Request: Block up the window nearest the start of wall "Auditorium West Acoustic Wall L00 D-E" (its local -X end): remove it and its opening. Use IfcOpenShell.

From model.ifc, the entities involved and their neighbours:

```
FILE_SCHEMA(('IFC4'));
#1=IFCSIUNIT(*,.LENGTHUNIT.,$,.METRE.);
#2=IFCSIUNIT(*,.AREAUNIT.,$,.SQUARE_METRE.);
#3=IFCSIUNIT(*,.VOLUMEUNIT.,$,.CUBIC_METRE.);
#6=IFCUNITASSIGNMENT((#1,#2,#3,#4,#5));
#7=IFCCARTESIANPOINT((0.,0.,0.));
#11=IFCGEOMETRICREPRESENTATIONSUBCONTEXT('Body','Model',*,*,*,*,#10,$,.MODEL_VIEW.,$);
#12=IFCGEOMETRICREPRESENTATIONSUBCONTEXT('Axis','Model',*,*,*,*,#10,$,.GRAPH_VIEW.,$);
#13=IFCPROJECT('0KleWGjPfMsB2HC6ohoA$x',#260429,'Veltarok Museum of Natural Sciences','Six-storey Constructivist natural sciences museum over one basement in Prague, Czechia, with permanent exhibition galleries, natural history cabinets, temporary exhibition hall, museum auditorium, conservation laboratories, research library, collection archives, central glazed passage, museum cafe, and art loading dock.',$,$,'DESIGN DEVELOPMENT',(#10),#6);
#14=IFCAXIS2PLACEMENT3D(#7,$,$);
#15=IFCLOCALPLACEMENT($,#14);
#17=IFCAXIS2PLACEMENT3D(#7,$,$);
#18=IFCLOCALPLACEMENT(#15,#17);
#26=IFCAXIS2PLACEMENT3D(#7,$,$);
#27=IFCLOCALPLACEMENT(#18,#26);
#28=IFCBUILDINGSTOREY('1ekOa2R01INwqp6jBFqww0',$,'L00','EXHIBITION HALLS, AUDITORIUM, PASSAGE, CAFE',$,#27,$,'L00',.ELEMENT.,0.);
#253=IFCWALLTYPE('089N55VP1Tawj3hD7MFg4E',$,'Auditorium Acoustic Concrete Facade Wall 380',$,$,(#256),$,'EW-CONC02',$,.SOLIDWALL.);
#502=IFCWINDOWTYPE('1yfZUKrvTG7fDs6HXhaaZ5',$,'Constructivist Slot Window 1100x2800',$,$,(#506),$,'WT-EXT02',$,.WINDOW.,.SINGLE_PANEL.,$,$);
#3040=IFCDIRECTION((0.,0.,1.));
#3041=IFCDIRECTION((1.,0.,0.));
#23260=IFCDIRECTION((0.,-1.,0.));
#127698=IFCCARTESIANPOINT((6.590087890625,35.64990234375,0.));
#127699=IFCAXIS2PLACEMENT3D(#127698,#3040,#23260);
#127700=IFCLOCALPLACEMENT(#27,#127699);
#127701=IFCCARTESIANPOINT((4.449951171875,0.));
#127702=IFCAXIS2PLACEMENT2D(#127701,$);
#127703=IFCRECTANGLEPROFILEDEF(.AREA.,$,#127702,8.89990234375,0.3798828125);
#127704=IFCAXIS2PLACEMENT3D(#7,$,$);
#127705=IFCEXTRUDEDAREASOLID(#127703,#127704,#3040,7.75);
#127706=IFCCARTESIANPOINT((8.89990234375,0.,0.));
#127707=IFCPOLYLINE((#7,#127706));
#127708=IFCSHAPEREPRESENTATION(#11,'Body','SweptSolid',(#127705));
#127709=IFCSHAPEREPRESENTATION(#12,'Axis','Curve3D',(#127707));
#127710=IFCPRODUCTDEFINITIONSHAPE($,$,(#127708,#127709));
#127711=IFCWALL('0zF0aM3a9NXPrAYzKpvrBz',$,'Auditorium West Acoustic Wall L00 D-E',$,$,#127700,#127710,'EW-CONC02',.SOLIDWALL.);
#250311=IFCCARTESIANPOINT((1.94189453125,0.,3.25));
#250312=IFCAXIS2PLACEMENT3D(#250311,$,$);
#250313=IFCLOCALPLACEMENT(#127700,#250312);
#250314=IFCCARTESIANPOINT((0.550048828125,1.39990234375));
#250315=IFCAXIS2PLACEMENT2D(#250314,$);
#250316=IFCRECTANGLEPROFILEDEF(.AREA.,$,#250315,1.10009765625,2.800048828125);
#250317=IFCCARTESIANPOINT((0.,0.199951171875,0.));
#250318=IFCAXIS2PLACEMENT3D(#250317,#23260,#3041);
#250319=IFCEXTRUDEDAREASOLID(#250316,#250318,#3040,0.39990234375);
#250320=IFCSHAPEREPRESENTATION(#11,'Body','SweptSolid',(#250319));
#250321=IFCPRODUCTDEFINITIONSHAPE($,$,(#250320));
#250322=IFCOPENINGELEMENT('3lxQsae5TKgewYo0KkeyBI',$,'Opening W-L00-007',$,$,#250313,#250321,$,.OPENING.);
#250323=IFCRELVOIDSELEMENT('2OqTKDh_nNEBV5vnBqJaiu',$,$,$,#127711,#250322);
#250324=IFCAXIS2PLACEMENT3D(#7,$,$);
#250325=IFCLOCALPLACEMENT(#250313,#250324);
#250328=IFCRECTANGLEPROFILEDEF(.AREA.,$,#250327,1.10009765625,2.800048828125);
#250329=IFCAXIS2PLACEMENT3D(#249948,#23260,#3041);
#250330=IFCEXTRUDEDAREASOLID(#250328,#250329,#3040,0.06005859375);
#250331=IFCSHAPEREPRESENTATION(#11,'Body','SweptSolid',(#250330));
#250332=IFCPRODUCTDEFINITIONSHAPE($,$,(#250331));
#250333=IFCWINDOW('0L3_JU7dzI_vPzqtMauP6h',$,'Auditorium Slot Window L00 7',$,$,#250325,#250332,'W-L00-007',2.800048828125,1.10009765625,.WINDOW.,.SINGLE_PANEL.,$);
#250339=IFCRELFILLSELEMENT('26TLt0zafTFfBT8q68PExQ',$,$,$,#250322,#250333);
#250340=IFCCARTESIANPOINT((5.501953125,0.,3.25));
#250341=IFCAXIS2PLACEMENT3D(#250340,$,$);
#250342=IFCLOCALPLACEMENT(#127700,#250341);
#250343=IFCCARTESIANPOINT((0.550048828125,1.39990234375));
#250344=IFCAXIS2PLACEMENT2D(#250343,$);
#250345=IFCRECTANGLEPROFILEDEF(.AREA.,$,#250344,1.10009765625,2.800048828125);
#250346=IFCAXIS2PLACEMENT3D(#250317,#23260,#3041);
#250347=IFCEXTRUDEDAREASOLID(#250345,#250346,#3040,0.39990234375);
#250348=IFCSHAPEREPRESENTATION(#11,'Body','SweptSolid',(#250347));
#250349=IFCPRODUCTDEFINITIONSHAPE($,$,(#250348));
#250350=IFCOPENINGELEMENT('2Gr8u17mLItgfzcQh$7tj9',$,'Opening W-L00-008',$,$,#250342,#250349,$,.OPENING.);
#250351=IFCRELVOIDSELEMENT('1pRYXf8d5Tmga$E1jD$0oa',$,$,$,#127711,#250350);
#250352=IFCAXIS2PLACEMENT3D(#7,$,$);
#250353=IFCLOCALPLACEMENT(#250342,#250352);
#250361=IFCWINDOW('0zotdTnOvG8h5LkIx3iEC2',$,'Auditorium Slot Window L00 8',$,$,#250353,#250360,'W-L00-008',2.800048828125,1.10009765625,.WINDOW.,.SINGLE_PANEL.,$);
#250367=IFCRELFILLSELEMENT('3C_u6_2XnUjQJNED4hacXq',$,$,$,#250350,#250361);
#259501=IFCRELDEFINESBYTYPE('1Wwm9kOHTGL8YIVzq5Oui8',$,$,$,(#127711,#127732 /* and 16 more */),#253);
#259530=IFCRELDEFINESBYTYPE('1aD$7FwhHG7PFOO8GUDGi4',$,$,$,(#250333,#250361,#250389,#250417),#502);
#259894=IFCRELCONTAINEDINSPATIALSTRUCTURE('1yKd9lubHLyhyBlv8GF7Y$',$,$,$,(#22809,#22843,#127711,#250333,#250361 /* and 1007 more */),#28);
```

```python
import ifcopenshell
import ifcopenshell.api.feature
import ifcopenshell.api.root
import ifcopenshell.geom
import ifcopenshell.util.shape

model = ifcopenshell.open("model.ifc")
settings = ifcopenshell.geom.settings()


def volume(element):
    """Net volume in cubic metres, openings subtracted."""
    shape = ifcopenshell.geom.create_shape(settings, element)
    return ifcopenshell.util.shape.get_volume(shape.geometry)


window = model.by_id(250333)
opening = window.FillsVoids[0].RelatingOpeningElement
wall = opening.VoidsElements[0].RelatingBuildingElement
before = volume(wall)

ifcopenshell.api.root.remove_product(model, product=window)
ifcopenshell.api.feature.remove_feature(model, feature=opening)

after = volume(wall)

print(f"wall volume {before:.3f} -> {after:.3f} m3")

model.write("model_v2.ifc")
```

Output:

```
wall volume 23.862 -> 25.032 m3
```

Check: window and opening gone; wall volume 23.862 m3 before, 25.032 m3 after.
